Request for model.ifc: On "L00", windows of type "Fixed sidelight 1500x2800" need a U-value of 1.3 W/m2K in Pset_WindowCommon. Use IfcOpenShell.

First a look at what the model holds.

```python
import ifcopenshell
import ifcopenshell.util.element

model = ifcopenshell.open("model.ifc")
print(model.schema)
storey = next(s for s in model.by_type("IfcBuildingStorey") if s.Name == "L00")
windows = [e for e in ifcopenshell.util.element.get_decomposition(storey) if e.is_a("IfcWindow")]
seen = {}
for e in windows:
    element_type = ifcopenshell.util.element.get_type(e)
    key = (element_type.Name if element_type != e and element_type else None, ifcopenshell.util.element.get_pset(e, "Pset_WindowCommon", "ThermalTransmittance"))
    seen[key] = seen.get(key, 0) + 1
for (name, value), count in sorted(seen.items(), key=str):
    print(count, "x", name, "|", value)
```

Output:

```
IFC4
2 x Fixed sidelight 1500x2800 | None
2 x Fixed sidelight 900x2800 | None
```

```python
import ifcopenshell
import ifcopenshell.api.pset
import ifcopenshell.util.element

model = ifcopenshell.open("model.ifc")

storey = next(s for s in model.by_type("IfcBuildingStorey") if s.Name == "L00")
windows = [e for e in ifcopenshell.util.element.get_decomposition(storey) if e.is_a("IfcWindow")]

count = 0
for e in windows:
    element_type = ifcopenshell.util.element.get_type(e)
    if element_type in (None, e) or element_type.Name != "Fixed sidelight 1500x2800":
        continue
    # add_pset returns the element's existing set when there is one.
    pset = ifcopenshell.api.pset.add_pset(model, product=e, name="Pset_WindowCommon")
    ifcopenshell.api.pset.edit_pset(model, pset=pset, properties={"ThermalTransmittance": 1.3})
    count += 1

print(count, "windows updated")

model.write("model_rev.ifc")
```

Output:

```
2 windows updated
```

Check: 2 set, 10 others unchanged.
